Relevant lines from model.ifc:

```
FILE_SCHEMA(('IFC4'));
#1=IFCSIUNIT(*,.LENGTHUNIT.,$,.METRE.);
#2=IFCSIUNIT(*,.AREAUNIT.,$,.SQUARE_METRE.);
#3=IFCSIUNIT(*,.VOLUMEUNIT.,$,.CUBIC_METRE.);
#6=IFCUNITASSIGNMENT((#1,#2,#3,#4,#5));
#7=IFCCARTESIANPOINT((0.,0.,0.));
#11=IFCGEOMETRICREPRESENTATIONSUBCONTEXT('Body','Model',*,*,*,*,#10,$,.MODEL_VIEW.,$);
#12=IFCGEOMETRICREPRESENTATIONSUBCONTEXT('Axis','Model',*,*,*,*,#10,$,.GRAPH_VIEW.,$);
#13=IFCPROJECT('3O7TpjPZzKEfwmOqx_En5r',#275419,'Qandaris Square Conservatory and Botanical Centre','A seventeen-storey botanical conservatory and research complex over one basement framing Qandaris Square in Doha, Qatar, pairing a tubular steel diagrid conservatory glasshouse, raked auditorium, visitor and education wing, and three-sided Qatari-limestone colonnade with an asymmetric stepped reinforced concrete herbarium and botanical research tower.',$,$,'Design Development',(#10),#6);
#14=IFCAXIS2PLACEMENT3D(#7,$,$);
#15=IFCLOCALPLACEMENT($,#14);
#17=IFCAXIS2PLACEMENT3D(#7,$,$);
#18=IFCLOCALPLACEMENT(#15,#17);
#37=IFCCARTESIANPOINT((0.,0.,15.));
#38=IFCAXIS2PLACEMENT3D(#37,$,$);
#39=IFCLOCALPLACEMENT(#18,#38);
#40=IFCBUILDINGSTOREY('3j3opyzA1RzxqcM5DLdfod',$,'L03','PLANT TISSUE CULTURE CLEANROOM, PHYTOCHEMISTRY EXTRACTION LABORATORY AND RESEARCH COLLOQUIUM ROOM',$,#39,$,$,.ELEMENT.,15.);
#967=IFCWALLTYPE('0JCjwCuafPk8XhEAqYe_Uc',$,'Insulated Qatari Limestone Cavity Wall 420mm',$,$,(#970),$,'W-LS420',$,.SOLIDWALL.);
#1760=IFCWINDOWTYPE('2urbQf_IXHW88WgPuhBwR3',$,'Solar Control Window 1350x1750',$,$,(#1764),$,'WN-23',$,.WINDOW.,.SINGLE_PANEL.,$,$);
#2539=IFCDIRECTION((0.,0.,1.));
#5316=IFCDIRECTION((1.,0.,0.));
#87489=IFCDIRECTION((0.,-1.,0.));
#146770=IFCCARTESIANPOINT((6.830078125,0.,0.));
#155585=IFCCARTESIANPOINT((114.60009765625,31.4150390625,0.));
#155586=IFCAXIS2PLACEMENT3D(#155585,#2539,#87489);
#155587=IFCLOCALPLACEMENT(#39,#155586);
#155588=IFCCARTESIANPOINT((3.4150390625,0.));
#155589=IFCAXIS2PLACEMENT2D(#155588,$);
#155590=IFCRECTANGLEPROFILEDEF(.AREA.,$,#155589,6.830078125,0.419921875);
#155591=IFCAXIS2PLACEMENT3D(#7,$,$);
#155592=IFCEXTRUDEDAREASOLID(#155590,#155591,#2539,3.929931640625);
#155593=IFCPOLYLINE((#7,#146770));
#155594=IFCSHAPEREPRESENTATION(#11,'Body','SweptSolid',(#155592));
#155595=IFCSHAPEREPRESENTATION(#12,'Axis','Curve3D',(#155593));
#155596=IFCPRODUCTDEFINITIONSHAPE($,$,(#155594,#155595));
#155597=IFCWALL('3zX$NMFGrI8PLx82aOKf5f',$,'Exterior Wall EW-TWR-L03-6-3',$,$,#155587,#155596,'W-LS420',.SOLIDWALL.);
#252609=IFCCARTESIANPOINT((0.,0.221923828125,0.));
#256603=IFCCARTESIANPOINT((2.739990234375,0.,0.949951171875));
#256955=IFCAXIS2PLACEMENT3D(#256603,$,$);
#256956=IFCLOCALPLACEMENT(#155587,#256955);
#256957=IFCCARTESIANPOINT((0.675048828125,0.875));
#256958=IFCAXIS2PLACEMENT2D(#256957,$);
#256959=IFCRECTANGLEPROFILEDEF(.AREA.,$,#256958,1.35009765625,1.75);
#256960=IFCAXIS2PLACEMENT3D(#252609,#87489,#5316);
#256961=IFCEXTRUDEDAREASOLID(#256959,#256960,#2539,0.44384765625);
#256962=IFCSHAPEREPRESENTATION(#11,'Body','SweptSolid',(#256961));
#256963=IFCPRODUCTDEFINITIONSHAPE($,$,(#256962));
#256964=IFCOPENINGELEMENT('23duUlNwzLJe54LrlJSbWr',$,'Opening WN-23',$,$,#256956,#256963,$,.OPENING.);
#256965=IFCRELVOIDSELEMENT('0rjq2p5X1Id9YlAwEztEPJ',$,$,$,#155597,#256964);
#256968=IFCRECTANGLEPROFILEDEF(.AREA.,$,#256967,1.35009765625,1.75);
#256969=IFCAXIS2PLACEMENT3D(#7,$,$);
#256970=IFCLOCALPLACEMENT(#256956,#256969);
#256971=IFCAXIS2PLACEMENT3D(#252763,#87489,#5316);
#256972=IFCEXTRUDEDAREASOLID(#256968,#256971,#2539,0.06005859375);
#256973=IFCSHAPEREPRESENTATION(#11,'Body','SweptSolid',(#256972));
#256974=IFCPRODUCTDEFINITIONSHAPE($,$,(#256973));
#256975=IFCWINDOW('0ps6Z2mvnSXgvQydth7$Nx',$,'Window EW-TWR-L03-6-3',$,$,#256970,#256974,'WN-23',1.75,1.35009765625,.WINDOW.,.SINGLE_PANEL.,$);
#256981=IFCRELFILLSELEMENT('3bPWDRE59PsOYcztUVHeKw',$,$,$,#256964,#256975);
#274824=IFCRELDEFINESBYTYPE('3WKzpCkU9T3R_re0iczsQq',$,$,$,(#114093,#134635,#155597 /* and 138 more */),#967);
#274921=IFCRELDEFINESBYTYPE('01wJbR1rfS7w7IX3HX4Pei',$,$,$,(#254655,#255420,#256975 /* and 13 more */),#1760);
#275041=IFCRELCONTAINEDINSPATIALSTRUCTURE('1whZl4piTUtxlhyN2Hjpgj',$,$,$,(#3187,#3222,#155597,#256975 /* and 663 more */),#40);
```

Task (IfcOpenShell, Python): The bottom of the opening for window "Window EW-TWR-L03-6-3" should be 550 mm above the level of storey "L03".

```python
import numpy as np
import ifcopenshell
import ifcopenshell.api.geometry
import ifcopenshell.geom
import ifcopenshell.util.element
import ifcopenshell.util.placement
import ifcopenshell.util.shape
import ifcopenshell.util.unit

model = ifcopenshell.open("model.ifc")
unit_scale = ifcopenshell.util.unit.calculate_unit_scale(model)

window = model.by_guid("0ps6Z2mvnSXgvQydth7$Nx")
opening = window.FillsVoids[0].RelatingOpeningElement
storey = ifcopenshell.util.element.get_container(window, ifc_class="IfcBuildingStorey")
level = ifcopenshell.util.placement.get_local_placement(storey.ObjectPlacement)[2, 3]

# The opening's origin need not be at the sill, so measure its lowest point.
shape = ifcopenshell.geom.create_shape(ifcopenshell.geom.settings(), opening)
bottom = ifcopenshell.util.shape.get_shape_bottom_elevation(shape, shape.geometry) / unit_scale
dz = level + 0.55 / unit_scale - bottom

shift = np.array([0.0, 0.0, dz])
# The window is placed relative to its opening, so it follows when the opening moves.
matrix = ifcopenshell.util.placement.get_local_placement(opening.ObjectPlacement)
matrix[:3, 3] += shift
ifcopenshell.api.geometry.edit_object_placement(
    model, product=opening, matrix=matrix, is_si=False, should_transform_children=True
)

print(f"moved by {dz * unit_scale:+.3f} m")

model.write("model-out.ifc")
```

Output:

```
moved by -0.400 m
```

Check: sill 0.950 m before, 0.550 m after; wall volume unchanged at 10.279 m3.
